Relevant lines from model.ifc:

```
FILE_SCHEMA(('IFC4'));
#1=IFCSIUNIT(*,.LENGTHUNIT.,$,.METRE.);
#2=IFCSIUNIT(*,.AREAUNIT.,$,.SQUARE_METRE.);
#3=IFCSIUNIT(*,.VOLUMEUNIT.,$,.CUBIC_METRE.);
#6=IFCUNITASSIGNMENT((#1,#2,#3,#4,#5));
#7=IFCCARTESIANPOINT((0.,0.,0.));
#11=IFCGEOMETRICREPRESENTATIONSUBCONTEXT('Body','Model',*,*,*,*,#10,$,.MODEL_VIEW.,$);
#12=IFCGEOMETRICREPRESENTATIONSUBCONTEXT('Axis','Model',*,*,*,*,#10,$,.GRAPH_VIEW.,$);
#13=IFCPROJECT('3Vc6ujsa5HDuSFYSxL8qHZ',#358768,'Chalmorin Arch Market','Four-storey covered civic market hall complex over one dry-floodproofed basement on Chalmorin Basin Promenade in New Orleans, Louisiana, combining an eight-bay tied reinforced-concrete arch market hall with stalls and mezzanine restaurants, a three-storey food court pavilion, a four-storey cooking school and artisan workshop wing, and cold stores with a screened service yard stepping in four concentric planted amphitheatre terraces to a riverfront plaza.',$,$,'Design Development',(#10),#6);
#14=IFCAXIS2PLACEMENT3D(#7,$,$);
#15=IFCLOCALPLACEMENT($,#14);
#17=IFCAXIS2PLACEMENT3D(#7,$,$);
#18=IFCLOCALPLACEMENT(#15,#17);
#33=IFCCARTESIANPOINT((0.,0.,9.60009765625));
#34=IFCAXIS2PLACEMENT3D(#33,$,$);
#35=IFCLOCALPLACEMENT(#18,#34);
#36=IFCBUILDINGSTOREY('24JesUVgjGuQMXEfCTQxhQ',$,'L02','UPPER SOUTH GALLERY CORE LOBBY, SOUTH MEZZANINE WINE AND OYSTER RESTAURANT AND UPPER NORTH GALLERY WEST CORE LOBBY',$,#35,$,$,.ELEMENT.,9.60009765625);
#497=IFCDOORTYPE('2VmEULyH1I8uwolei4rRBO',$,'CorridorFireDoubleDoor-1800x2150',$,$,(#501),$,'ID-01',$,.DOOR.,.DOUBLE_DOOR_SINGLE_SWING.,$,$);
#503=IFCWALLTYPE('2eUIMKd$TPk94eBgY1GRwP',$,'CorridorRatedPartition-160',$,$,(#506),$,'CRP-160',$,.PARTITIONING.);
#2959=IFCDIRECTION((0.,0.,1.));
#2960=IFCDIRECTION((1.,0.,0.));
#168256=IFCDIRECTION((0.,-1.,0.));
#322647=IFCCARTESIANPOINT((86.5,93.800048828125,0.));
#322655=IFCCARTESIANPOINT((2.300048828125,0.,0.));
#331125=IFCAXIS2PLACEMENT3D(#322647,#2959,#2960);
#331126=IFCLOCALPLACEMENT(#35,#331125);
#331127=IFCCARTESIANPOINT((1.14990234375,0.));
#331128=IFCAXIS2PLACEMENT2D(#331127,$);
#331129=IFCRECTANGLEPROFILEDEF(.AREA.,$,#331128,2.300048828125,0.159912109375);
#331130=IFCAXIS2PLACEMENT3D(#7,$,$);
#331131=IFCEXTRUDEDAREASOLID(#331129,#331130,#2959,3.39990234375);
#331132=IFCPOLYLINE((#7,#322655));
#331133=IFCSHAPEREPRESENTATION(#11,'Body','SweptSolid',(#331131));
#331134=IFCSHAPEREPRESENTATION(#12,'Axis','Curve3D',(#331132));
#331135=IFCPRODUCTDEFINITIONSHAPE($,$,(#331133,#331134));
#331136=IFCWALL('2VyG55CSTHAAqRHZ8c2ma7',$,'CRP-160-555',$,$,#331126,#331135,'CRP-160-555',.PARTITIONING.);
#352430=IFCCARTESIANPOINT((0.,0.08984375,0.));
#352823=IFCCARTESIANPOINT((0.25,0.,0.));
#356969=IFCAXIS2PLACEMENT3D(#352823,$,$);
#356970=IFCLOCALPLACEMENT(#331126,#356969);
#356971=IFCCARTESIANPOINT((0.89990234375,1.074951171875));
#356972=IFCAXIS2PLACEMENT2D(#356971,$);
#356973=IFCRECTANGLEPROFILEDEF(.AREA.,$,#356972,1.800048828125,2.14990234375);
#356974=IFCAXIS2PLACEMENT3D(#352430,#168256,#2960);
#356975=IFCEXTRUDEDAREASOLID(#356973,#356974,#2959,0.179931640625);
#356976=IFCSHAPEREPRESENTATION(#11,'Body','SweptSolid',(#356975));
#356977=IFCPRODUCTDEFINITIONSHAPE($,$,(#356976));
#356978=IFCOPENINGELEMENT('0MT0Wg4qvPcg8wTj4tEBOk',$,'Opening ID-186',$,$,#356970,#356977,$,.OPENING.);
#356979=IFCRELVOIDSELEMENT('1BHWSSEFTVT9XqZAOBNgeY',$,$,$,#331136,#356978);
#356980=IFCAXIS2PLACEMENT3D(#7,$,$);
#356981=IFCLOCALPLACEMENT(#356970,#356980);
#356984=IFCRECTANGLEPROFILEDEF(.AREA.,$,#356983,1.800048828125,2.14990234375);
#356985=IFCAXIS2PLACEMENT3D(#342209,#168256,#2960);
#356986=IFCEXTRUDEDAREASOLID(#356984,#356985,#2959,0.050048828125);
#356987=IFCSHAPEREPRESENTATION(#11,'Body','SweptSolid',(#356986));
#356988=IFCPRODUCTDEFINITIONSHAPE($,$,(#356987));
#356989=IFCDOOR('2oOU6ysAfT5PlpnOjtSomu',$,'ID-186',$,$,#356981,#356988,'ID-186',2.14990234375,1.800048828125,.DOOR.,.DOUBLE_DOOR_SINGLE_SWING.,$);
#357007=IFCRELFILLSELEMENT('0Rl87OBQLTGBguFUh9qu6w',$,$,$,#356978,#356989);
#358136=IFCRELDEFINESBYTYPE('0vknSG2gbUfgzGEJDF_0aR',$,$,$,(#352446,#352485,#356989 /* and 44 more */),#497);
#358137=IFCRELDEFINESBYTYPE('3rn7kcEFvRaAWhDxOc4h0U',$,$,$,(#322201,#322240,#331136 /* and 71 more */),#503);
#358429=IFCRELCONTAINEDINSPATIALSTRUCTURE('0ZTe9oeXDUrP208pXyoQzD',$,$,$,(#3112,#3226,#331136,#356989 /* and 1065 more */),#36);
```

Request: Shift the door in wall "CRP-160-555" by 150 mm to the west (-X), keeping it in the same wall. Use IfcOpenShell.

```python
import ifcopenshell
import ifcopenshell.api.geometry
import ifcopenshell.util.placement

model = ifcopenshell.open("model.ifc")

door = model.by_guid("2oOU6ysAfT5PlpnOjtSomu")
opening = door.FillsVoids[0].RelatingOpeningElement
wall = opening.VoidsElements[0].RelatingBuildingElement

wall_matrix = ifcopenshell.util.placement.get_local_placement(wall.ObjectPlacement)
shift = wall_matrix[:3, 0] * -0.15
before = ifcopenshell.util.placement.get_local_placement(door.ObjectPlacement)[:3, 3].copy()

# The door is placed relative to its opening, so it follows when the opening moves.
matrix = ifcopenshell.util.placement.get_local_placement(opening.ObjectPlacement)
matrix[:3, 3] += shift
ifcopenshell.api.geometry.edit_object_placement(
    model, product=opening, matrix=matrix, is_si=False, should_transform_children=True
)

after = ifcopenshell.util.placement.get_local_placement(door.ObjectPlacement)[:3, 3]
print("door moved by", (after - before).round(3) + 0.0)

model.write("model_updated.ifc")
```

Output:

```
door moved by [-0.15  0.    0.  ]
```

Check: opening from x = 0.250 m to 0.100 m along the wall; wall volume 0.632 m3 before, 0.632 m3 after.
